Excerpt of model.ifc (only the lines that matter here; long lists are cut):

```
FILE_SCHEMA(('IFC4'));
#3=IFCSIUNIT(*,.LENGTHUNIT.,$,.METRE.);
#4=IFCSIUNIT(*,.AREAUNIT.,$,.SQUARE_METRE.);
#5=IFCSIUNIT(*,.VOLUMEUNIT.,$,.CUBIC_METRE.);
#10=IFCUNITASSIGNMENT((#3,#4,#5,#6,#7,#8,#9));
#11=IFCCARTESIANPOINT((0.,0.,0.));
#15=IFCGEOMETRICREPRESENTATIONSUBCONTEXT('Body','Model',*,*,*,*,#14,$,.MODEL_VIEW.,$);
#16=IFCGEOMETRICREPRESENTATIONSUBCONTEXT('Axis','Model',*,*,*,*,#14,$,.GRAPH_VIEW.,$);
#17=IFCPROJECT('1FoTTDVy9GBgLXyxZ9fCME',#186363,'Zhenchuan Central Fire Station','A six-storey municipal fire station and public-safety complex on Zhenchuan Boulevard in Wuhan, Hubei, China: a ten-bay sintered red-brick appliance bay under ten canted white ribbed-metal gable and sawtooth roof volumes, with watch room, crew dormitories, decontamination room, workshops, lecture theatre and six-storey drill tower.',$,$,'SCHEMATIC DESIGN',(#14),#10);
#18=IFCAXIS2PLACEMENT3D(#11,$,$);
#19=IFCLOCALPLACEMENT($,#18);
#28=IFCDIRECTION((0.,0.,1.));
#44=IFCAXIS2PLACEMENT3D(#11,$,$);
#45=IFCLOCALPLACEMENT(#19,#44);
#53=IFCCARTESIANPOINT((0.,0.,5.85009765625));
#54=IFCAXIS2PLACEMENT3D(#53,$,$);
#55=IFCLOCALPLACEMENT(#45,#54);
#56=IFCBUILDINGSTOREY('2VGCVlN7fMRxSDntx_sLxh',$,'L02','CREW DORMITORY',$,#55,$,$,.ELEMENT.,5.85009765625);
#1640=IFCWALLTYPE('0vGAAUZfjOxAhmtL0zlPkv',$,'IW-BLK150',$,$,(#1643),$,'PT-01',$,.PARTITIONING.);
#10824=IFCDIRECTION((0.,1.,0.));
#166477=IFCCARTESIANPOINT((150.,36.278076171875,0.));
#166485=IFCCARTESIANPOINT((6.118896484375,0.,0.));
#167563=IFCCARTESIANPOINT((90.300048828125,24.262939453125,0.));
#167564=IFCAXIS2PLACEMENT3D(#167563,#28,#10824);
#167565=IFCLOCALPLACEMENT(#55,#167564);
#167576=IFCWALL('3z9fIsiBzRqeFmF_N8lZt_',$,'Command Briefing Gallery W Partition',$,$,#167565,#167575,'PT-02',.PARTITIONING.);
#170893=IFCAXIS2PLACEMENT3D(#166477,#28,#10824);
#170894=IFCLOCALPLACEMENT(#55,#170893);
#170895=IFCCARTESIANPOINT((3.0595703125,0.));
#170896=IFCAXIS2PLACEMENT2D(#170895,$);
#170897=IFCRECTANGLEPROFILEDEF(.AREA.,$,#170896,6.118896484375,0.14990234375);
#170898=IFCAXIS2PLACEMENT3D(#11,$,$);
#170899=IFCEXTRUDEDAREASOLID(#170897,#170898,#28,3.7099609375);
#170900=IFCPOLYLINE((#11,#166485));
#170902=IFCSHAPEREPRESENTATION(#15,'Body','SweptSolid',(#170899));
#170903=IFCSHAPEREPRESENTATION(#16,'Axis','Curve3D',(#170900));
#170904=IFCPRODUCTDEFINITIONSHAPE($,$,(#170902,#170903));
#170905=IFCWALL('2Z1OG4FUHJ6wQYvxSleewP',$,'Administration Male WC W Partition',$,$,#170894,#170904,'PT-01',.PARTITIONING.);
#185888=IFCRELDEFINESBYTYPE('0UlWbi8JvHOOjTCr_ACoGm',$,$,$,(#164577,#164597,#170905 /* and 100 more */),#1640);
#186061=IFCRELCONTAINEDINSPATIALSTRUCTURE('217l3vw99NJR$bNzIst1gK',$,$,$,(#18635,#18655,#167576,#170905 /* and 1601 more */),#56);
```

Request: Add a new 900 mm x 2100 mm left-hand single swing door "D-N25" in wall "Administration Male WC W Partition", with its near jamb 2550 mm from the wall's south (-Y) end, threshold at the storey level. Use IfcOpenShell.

```python
import numpy as np
import ifcopenshell
import ifcopenshell.api.feature
import ifcopenshell.api.geometry
import ifcopenshell.api.root
import ifcopenshell.api.spatial
import ifcopenshell.geom
import ifcopenshell.util.element
import ifcopenshell.util.placement
import ifcopenshell.util.representation
import ifcopenshell.util.shape
import ifcopenshell.util.unit

model = ifcopenshell.open("model.ifc")
unit_scale = ifcopenshell.util.unit.calculate_unit_scale(model)
settings = ifcopenshell.geom.settings()


def volume(element):
    """Net volume in cubic metres, openings subtracted."""
    shape = ifcopenshell.geom.create_shape(settings, element)
    return ifcopenshell.util.shape.get_volume(shape.geometry)


wall = model.by_id(170905)
storey = ifcopenshell.util.element.get_container(wall, ifc_class="IfcBuildingStorey")
context = ifcopenshell.util.representation.get_context(model, "Model", "Body", "MODEL_VIEW")
before = volume(wall)

width, height, from_end, sill = 0.9, 2.1, 2.55, 0.0  # metres

# The wall runs along its own X axis, and the end named is its -X end.
wall_shape = ifcopenshell.geom.create_shape(settings, wall)
x, y, z = ifcopenshell.util.shape.get_vertices(wall_shape.geometry).T
start = x.min() + from_end
face, thickness = float(y.min()), float(y.max() - y.min())
wall_matrix = ifcopenshell.util.placement.get_local_placement(wall.ObjectPlacement)
level = ifcopenshell.util.placement.get_local_placement(storey.ObjectPlacement)[2, 3]


def in_wall(x, y):
    """Placement at x, y metres in the wall's axes, at sill height."""
    matrix = wall_matrix.copy()
    matrix[:, 3] = wall_matrix @ np.array([x / unit_scale, y / unit_scale, 0.0, 1.0])
    matrix[2, 3] = level + sill / unit_scale
    return matrix


# Opening: a box that overshoots both wall faces by 50 mm.
opening = ifcopenshell.api.root.create_entity(model, ifc_class="IfcOpeningElement", predefined_type="OPENING")
box = ifcopenshell.api.geometry.add_wall_representation(
    model, context=context, length=width, height=height, thickness=thickness + 0.1
)
ifcopenshell.api.geometry.assign_representation(model, product=opening, representation=box)
ifcopenshell.api.geometry.edit_object_placement(model, product=opening, matrix=in_wall(start, face - 0.05), is_si=False)
ifcopenshell.api.feature.add_feature(model, feature=opening, element=wall)

door = ifcopenshell.api.root.create_entity(model, ifc_class="IfcDoor", name="D-N25", predefined_type="DOOR")
door.OverallWidth, door.OverallHeight = width / unit_scale, height / unit_scale
door.OperationType = "SINGLE_SWING_LEFT"
body = ifcopenshell.api.geometry.add_door_representation(
    model,
    context=context,
    overall_width=door.OverallWidth,
    overall_height=door.OverallHeight,
    operation_type="SINGLE_SWING_LEFT",
    lining_properties={"LiningDepth": thickness / unit_scale, "ThresholdDepth": thickness / unit_scale},
)
ifcopenshell.api.geometry.assign_representation(model, product=door, representation=body)
ifcopenshell.api.spatial.assign_container(model, products=[door], relating_structure=storey)
ifcopenshell.api.feature.add_filling(model, opening=opening, element=door)

# The lining spans the wall, so the door starts at the wall face.
ifcopenshell.api.geometry.edit_object_placement(model, product=door, matrix=in_wall(start, face), is_si=False)

after = volume(wall)

print(f"wall volume {before:.3f} -> {after:.3f} m3")

model.write("model_rev.ifc")
```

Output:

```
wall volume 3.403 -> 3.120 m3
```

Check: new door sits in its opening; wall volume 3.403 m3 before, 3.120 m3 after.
